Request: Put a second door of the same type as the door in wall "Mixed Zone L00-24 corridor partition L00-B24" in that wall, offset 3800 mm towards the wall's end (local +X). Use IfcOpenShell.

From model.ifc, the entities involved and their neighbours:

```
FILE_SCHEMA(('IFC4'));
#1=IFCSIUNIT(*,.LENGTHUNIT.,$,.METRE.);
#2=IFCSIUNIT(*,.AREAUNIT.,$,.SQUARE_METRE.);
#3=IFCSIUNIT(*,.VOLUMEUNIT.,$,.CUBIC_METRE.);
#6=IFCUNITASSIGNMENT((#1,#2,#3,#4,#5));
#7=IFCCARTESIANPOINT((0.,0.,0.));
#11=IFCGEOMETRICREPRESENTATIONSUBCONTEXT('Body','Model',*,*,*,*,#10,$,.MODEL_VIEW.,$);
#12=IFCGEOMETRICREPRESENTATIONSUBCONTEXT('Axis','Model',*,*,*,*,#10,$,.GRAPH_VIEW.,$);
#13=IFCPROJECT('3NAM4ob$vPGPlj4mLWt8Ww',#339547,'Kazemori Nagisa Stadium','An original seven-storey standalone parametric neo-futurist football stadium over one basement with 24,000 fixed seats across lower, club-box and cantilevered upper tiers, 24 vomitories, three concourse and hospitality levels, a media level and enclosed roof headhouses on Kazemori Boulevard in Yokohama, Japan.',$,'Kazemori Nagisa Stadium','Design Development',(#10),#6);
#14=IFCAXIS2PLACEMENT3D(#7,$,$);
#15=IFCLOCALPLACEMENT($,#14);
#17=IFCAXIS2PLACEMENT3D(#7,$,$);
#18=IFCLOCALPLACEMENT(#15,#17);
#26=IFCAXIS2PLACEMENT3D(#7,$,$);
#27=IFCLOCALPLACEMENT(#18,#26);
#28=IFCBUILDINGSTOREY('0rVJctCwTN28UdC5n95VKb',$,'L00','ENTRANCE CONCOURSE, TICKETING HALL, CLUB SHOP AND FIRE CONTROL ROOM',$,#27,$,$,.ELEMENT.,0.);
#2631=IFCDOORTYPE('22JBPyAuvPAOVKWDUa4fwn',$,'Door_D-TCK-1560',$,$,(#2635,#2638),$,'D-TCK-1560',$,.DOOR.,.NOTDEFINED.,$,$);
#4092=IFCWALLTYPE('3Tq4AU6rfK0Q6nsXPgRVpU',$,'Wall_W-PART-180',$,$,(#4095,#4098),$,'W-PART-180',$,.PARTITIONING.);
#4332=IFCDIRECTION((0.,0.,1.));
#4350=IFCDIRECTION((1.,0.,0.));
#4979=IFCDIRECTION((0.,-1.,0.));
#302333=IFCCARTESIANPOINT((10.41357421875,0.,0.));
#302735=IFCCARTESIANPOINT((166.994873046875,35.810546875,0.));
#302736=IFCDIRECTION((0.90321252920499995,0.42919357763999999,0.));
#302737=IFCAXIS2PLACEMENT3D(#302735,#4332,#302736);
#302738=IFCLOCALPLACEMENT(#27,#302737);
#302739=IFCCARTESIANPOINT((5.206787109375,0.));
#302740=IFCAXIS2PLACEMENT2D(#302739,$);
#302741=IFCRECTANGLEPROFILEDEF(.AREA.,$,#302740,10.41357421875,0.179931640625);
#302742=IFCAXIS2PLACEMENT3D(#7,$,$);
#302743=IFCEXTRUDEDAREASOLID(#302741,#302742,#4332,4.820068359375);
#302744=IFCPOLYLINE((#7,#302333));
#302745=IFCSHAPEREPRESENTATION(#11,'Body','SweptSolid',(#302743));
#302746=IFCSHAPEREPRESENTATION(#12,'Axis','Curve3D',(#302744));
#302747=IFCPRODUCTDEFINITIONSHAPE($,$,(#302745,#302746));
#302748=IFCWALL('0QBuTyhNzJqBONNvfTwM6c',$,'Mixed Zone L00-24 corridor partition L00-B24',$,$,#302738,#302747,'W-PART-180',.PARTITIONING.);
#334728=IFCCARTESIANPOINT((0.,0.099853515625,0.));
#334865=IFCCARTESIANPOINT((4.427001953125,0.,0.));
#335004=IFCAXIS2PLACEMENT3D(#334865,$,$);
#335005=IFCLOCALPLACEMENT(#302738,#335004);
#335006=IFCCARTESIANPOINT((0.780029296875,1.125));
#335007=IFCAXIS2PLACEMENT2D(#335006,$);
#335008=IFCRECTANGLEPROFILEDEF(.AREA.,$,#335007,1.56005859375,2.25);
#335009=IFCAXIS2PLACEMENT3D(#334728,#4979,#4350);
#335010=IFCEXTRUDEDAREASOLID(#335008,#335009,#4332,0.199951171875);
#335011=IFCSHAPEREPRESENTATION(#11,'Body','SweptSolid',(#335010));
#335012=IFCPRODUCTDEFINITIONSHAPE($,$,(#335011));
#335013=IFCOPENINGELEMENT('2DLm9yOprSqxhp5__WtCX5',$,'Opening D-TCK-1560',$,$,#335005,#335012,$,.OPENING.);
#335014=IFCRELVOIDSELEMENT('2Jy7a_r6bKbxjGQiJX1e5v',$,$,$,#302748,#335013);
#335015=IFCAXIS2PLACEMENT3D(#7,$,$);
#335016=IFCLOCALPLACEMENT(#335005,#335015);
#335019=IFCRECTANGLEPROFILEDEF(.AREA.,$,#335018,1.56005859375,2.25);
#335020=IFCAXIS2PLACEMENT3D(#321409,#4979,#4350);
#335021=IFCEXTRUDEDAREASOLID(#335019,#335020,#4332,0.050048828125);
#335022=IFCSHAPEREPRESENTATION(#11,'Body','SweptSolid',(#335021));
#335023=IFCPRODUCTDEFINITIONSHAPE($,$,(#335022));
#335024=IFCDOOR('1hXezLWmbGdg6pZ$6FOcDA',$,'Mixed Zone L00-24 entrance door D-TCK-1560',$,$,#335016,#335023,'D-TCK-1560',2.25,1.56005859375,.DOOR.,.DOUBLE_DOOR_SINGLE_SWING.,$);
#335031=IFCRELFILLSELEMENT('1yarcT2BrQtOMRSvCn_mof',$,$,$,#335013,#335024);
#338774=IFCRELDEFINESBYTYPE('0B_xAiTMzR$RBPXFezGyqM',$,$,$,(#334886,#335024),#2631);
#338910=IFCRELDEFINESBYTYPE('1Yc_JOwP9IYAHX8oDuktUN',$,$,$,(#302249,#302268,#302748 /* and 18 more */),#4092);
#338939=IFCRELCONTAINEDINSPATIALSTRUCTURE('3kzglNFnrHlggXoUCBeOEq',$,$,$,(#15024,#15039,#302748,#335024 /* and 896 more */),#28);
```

```python
import ifcopenshell
import ifcopenshell.api.feature
import ifcopenshell.api.geometry
import ifcopenshell.api.root
import ifcopenshell.geom
import ifcopenshell.util.element
import ifcopenshell.util.placement
import ifcopenshell.util.shape
import ifcopenshell.util.unit

model = ifcopenshell.open("model.ifc")
unit_scale = ifcopenshell.util.unit.calculate_unit_scale(model)
settings = ifcopenshell.geom.settings()


def volume(element):
    """Net volume in cubic metres, openings subtracted."""
    shape = ifcopenshell.geom.create_shape(settings, element)
    return ifcopenshell.util.shape.get_volume(shape.geometry)


door = model.by_id(335024)
opening = door.FillsVoids[0].RelatingOpeningElement
wall = opening.VoidsElements[0].RelatingBuildingElement
before = volume(wall)
shift = ifcopenshell.util.placement.get_local_placement(wall.ObjectPlacement)[:3, 0] * 3.8 / unit_scale

# copy_class copies the void relationship, type, container and properties, but no geometry.
new_opening = ifcopenshell.api.root.copy_class(model, product=opening)
new_opening.Representation = ifcopenshell.util.element.copy_deep(
    model, opening.Representation, exclude=["IfcGeometricRepresentationContext", "IfcRepresentationMap"]
)
new_door = ifcopenshell.api.root.copy_class(model, product=door)
new_door.Representation = ifcopenshell.util.element.copy_deep(
    model, door.Representation, exclude=["IfcGeometricRepresentationContext", "IfcRepresentationMap"]
)
new_door.Tag = None
ifcopenshell.api.feature.add_filling(model, opening=new_opening, element=new_door)

for old, new in ((opening, new_opening), (door, new_door)):
    matrix = ifcopenshell.util.placement.get_local_placement(old.ObjectPlacement)
    matrix[:3, 3] += shift
    ifcopenshell.api.geometry.edit_object_placement(model, product=new, matrix=matrix, is_si=False)

after = volume(wall)

print(f"wall volume {before:.3f} -> {after:.3f} m3")

model.write("model_v2.ifc")
```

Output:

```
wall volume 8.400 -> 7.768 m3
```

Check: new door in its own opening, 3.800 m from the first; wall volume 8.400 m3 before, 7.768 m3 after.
